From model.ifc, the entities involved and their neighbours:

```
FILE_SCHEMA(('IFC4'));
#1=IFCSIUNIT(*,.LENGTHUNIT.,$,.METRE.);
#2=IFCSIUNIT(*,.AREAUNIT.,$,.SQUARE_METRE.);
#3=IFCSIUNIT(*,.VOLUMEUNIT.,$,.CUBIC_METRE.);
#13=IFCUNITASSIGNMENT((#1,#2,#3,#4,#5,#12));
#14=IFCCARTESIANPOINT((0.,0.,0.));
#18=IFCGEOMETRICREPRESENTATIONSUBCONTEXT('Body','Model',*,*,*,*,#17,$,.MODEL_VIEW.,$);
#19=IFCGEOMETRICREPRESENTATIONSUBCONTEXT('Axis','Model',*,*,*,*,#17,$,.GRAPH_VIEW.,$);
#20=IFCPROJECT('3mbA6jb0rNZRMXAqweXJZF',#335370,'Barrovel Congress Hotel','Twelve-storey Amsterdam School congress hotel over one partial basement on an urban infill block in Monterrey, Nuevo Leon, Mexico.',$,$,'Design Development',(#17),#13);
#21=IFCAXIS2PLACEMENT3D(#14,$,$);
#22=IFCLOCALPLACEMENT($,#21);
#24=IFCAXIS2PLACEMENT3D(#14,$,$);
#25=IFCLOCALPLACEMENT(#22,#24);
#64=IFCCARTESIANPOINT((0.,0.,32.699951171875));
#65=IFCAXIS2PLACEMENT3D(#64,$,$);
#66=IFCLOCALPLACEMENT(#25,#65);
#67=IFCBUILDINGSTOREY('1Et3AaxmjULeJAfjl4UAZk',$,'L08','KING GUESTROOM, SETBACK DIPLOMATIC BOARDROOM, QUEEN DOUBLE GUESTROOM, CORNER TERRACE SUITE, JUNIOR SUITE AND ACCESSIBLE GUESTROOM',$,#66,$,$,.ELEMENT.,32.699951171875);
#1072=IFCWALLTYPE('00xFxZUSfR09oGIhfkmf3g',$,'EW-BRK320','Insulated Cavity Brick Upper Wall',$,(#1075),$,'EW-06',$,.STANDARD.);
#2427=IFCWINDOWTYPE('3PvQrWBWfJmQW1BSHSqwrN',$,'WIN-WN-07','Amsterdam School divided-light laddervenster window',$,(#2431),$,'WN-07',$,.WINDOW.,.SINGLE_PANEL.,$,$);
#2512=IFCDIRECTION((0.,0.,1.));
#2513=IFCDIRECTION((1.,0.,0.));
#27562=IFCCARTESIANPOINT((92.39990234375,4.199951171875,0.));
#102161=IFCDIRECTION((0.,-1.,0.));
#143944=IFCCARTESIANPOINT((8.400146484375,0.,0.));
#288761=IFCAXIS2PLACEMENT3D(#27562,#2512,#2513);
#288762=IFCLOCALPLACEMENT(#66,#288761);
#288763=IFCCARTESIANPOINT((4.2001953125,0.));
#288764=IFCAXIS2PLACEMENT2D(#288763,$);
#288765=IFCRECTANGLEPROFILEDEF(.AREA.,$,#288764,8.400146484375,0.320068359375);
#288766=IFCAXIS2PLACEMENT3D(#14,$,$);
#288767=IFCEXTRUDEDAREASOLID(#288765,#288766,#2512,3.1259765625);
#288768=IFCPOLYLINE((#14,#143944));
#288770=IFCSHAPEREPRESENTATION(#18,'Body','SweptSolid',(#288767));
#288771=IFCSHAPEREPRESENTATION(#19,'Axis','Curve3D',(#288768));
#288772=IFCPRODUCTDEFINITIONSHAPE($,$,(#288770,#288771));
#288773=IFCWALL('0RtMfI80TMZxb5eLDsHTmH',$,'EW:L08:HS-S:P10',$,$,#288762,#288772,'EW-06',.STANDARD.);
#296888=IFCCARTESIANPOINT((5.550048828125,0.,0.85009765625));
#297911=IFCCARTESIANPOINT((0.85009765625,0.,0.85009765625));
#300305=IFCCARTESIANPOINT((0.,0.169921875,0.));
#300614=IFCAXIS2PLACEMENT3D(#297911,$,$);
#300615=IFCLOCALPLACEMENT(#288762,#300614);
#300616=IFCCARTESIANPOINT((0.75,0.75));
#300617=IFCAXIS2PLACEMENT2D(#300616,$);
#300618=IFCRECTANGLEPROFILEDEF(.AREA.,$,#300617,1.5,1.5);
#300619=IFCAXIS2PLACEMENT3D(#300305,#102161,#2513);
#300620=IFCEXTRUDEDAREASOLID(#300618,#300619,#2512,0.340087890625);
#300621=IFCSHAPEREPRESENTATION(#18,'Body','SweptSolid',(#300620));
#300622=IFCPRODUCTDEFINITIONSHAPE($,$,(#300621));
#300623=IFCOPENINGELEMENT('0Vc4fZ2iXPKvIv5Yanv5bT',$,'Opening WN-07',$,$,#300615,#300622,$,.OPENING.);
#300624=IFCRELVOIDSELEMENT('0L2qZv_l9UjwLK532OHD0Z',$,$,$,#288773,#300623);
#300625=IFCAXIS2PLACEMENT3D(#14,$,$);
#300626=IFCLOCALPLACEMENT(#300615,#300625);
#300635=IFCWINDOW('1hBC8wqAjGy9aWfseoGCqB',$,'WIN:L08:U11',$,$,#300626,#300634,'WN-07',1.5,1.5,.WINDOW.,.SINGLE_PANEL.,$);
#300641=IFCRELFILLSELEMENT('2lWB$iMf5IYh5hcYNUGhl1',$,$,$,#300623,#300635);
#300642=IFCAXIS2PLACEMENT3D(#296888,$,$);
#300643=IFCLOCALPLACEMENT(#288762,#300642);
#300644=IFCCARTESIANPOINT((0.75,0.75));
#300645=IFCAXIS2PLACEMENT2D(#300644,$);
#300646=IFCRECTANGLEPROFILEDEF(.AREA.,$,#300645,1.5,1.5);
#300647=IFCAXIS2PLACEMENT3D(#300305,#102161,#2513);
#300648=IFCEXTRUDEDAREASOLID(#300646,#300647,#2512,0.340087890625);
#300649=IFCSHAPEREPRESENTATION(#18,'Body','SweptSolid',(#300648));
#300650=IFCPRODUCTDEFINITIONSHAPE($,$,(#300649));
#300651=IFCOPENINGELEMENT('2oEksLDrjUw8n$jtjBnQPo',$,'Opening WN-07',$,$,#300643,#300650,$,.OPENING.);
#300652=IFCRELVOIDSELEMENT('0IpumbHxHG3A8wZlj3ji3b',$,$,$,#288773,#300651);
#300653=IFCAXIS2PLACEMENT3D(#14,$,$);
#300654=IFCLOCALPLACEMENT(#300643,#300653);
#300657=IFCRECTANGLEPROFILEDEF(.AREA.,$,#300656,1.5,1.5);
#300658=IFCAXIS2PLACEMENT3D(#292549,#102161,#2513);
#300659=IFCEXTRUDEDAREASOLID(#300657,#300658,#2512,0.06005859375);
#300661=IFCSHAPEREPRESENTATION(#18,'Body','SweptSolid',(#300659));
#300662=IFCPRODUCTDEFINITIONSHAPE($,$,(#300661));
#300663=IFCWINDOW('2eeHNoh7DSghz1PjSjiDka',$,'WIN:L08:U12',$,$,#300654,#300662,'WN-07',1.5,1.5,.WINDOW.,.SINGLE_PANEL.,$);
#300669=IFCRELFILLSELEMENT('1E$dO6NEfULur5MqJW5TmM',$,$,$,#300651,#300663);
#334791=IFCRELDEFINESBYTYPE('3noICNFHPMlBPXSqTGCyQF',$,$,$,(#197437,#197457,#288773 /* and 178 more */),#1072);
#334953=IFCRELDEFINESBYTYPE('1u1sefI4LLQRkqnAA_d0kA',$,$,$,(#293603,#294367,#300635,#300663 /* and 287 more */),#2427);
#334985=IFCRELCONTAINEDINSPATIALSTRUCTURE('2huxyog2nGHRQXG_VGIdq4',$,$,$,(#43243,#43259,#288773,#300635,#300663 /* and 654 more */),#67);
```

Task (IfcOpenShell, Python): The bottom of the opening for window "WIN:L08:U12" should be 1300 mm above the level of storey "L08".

```python
import numpy as np
import ifcopenshell
import ifcopenshell.api.geometry
import ifcopenshell.geom
import ifcopenshell.util.element
import ifcopenshell.util.placement
import ifcopenshell.util.shape
import ifcopenshell.util.unit

model = ifcopenshell.open("model.ifc")
unit_scale = ifcopenshell.util.unit.calculate_unit_scale(model)

window = model.by_guid("2eeHNoh7DSghz1PjSjiDka")
opening = window.FillsVoids[0].RelatingOpeningElement
storey = ifcopenshell.util.element.get_container(window, ifc_class="IfcBuildingStorey")
level = ifcopenshell.util.placement.get_local_placement(storey.ObjectPlacement)[2, 3]

# The opening's origin need not be at the sill, so measure its lowest point.
shape = ifcopenshell.geom.create_shape(ifcopenshell.geom.settings(), opening)
bottom = ifcopenshell.util.shape.get_shape_bottom_elevation(shape, shape.geometry) / unit_scale
dz = level + 1.3 / unit_scale - bottom

shift = np.array([0.0, 0.0, dz])
# The window is placed relative to its opening, so it follows when the opening moves.
matrix = ifcopenshell.util.placement.get_local_placement(opening.ObjectPlacement)
matrix[:3, 3] += shift
ifcopenshell.api.geometry.edit_object_placement(
    model, product=opening, matrix=matrix, is_si=False, should_transform_children=True
)

print(f"moved by {dz * unit_scale:+.3f} m")

model.write("model_v2.ifc")
```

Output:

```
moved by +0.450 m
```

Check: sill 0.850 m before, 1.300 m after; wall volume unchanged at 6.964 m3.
